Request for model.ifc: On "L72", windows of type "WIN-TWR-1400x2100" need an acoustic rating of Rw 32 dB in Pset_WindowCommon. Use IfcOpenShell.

First a look at what the model holds.

```python
import ifcopenshell
import ifcopenshell.util.element

model = ifcopenshell.open("model.ifc")
print(model.schema)
storey = next(s for s in model.by_type("IfcBuildingStorey") if s.Name == "L72")
windows = [e for e in ifcopenshell.util.element.get_decomposition(storey) if e.is_a("IfcWindow")]
seen = {}
for e in windows:
    element_type = ifcopenshell.util.element.get_type(e)
    key = (element_type.Name if element_type != e and element_type else None, ifcopenshell.util.element.get_pset(e, "Pset_WindowCommon", "AcousticRating"))
    seen[key] = seen.get(key, 0) + 1
for (name, value), count in sorted(seen.items(), key=str):
    print(count, "x", name, "|", value)
```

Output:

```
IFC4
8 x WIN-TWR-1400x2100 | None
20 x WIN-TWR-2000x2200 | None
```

```python
import ifcopenshell
import ifcopenshell.api.pset
import ifcopenshell.util.element

model = ifcopenshell.open("model.ifc")

storey = next(s for s in model.by_type("IfcBuildingStorey") if s.Name == "L72")
windows = [e for e in ifcopenshell.util.element.get_decomposition(storey) if e.is_a("IfcWindow")]

count = 0
for e in windows:
    element_type = ifcopenshell.util.element.get_type(e)
    if element_type in (None, e) or element_type.Name != "WIN-TWR-1400x2100":
        continue
    found = ifcopenshell.util.element.get_pset(e, "Pset_WindowCommon", should_inherit=False)
    if found:
        pset = model.by_id(found["id"])
        if len(ifcopenshell.util.element.get_elements_by_pset(pset)) > 1:
            pset = ifcopenshell.api.pset.unshare_pset(model, products=[e], pset=pset)[0]
    else:
        pset = ifcopenshell.api.pset.add_pset(model, product=e, name="Pset_WindowCommon")
    ifcopenshell.api.pset.edit_pset(model, pset=pset, properties={"AcousticRating": "Rw 32 dB"})
    count += 1

print(count, "windows updated")

model.write("model_updated.ifc")
```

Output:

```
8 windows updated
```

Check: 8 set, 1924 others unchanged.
